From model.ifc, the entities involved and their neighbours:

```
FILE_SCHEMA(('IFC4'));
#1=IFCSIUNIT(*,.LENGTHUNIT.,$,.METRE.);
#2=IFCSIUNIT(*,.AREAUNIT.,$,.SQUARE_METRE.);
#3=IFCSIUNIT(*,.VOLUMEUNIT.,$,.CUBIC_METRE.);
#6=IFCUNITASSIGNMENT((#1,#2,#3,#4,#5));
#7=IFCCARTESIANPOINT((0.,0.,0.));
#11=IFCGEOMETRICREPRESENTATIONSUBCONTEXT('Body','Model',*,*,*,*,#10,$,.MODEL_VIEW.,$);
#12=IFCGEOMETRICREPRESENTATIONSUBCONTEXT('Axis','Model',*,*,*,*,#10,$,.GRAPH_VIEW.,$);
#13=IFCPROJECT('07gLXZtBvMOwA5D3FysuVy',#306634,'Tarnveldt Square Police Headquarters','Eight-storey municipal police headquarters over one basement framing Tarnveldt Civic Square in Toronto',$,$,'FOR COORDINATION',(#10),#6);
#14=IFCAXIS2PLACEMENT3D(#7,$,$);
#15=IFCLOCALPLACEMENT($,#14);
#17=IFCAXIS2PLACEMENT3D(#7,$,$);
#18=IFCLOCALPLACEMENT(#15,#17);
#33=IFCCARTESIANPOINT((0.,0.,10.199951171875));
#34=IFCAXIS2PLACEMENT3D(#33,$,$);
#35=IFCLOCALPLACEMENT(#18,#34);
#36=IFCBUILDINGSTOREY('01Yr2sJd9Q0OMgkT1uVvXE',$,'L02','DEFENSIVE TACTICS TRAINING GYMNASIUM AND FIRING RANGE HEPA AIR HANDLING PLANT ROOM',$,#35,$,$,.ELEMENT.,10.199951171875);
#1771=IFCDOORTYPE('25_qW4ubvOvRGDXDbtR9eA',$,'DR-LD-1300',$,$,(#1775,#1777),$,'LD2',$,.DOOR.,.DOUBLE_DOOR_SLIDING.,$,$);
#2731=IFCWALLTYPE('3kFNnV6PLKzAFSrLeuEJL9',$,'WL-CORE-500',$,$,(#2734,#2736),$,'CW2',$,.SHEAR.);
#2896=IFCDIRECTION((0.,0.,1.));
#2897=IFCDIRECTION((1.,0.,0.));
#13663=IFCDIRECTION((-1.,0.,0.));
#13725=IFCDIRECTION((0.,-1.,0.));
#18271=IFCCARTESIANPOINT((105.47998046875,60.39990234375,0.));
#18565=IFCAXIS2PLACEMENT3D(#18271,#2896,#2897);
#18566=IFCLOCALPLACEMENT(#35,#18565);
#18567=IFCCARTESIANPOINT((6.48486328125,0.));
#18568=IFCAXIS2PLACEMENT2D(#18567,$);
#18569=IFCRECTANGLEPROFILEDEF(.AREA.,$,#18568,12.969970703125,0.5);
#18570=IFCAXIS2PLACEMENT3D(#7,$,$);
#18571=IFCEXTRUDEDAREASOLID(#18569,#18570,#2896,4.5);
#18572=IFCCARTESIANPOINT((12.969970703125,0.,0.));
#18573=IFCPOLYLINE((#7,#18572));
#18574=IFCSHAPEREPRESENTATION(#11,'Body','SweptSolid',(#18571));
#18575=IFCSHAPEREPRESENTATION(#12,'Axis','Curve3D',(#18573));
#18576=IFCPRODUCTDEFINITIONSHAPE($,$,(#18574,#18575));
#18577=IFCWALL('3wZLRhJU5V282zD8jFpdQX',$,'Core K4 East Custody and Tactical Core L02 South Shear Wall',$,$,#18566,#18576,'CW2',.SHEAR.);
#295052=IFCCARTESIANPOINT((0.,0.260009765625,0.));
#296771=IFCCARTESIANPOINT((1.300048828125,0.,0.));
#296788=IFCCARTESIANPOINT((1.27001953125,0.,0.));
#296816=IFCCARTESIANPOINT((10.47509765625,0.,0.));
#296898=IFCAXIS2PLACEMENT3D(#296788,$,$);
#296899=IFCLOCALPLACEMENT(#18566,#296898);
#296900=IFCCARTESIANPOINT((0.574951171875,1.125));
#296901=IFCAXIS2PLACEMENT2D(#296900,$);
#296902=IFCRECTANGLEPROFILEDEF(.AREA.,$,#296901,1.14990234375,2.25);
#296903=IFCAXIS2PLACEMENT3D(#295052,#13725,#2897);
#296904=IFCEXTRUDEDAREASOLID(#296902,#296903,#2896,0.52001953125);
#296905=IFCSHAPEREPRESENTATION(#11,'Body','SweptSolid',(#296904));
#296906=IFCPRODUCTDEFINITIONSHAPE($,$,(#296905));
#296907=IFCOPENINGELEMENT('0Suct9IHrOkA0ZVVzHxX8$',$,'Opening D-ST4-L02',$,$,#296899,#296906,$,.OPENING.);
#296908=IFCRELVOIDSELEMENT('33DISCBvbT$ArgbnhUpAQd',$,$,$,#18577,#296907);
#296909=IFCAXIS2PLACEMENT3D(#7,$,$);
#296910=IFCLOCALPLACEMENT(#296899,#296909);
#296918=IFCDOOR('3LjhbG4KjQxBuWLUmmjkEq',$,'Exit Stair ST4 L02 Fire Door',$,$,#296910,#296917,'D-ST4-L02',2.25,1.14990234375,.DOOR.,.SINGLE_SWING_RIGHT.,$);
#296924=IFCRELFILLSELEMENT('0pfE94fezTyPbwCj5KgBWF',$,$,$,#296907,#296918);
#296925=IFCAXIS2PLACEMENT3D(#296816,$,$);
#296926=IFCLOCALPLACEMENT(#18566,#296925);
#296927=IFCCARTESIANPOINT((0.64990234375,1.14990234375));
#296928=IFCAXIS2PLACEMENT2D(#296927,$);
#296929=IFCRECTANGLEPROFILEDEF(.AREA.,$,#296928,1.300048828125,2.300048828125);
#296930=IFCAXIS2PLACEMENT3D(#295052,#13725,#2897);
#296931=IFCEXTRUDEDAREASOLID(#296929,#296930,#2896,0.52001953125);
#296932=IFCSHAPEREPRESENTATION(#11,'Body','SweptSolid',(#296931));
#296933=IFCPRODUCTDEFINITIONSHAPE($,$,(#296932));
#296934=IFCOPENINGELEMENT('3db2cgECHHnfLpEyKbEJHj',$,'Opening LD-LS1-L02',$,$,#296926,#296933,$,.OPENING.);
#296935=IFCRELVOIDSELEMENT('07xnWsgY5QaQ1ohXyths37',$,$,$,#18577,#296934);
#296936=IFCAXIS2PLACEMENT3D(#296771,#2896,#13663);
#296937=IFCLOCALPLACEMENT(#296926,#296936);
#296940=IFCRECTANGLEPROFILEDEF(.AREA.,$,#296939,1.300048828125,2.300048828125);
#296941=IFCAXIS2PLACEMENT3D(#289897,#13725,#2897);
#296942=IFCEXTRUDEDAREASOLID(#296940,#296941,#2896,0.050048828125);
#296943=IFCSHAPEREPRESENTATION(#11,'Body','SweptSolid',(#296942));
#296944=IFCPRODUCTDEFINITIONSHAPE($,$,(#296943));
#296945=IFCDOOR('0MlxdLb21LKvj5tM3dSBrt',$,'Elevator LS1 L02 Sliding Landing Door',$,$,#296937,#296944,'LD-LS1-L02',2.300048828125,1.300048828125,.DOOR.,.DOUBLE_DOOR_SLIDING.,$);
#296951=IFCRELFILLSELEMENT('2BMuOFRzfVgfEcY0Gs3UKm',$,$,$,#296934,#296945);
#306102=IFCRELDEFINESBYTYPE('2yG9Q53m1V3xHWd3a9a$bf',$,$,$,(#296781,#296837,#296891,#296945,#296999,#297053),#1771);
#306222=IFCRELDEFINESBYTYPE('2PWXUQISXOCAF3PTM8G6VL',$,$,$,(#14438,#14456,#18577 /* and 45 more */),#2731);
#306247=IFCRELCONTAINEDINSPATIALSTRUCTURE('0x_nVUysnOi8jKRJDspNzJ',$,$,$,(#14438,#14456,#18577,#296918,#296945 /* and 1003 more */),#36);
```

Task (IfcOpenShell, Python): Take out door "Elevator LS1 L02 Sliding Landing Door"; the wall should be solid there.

```python
import ifcopenshell
import ifcopenshell.api.feature
import ifcopenshell.api.root
import ifcopenshell.geom
import ifcopenshell.util.shape

model = ifcopenshell.open("model.ifc")
settings = ifcopenshell.geom.settings()


def volume(element):
    """Net volume in cubic metres, openings subtracted."""
    shape = ifcopenshell.geom.create_shape(settings, element)
    return ifcopenshell.util.shape.get_volume(shape.geometry)


door = model.by_id(296945)
opening = door.FillsVoids[0].RelatingOpeningElement
wall = opening.VoidsElements[0].RelatingBuildingElement
before = volume(wall)

ifcopenshell.api.root.remove_product(model, product=door)
ifcopenshell.api.feature.remove_feature(model, feature=opening)

after = volume(wall)

print(f"wall volume {before:.3f} -> {after:.3f} m3")

model.write("model_rev.ifc")
```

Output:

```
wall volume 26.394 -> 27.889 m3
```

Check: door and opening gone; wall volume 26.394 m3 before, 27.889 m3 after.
